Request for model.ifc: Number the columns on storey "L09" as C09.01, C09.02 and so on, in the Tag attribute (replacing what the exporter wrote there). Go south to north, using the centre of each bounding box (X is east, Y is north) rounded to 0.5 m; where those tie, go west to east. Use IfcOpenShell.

First a look at what the model holds.

```python
import ifcopenshell
import ifcopenshell.util.element
import ifcopenshell.util.placement

model = ifcopenshell.open("model.ifc")
print(model.schema)
storey = next(s for s in model.by_type("IfcBuildingStorey") if s.Name == "L09")
columns = [e for e in ifcopenshell.util.element.get_decomposition(storey) if e.is_a("IfcColumn")]
for e in sorted(columns, key=lambda e: e.id()):
    origin = ifcopenshell.util.placement.get_local_placement(e.ObjectPlacement)[:3, 3]
    print(e.id(), e.Tag, e.Name, origin.round(2) + 0.0, sep=" | ")
```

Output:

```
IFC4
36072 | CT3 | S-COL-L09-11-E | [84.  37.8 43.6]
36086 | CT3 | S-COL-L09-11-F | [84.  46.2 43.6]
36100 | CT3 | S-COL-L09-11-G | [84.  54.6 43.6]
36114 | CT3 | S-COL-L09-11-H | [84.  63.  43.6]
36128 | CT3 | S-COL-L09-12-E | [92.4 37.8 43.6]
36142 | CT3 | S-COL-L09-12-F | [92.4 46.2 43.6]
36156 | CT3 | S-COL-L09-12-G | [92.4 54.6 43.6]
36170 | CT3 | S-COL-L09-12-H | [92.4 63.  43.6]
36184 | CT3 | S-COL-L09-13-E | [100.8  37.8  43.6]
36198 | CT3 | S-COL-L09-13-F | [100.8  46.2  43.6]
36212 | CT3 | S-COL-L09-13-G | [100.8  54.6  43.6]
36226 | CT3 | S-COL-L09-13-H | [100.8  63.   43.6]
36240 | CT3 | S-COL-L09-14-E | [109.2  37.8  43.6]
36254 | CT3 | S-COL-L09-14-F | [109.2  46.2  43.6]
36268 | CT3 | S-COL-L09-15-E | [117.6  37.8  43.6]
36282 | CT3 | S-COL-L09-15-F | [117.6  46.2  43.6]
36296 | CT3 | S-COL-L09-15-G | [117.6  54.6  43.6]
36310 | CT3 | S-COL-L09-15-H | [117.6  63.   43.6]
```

```python
import ifcopenshell
import ifcopenshell.geom
import ifcopenshell.util.element
import ifcopenshell.util.shape

model = ifcopenshell.open("model.ifc")
settings = ifcopenshell.geom.settings()
settings.set("use-world-coords", True)


def centre(element):
    shape = ifcopenshell.geom.create_shape(settings, element)
    return ifcopenshell.util.shape.get_bbox_centroid(shape.geometry)


storey = next(s for s in model.by_type("IfcBuildingStorey") if s.Name == "L09")
columns = [e for e in ifcopenshell.util.element.get_decomposition(storey) if e.is_a("IfcColumn")]

# Insertion points can sit at a corner or the storey origin, so sort by the geometry (in metres).
centres = {e: centre(e) for e in columns}
columns.sort(key=lambda e: (round(centres[e][1] / 0.5), centres[e][0]))

for i, e in enumerate(columns, start=1):
    number = f"C09.{i:02d}"
    e.Tag = number
    print(e.id(), number)

model.write("model-out.ifc")
```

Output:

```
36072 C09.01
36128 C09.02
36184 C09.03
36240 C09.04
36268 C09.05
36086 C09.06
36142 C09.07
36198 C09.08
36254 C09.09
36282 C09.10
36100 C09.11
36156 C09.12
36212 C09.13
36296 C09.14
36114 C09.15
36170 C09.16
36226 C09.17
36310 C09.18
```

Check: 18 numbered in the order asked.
